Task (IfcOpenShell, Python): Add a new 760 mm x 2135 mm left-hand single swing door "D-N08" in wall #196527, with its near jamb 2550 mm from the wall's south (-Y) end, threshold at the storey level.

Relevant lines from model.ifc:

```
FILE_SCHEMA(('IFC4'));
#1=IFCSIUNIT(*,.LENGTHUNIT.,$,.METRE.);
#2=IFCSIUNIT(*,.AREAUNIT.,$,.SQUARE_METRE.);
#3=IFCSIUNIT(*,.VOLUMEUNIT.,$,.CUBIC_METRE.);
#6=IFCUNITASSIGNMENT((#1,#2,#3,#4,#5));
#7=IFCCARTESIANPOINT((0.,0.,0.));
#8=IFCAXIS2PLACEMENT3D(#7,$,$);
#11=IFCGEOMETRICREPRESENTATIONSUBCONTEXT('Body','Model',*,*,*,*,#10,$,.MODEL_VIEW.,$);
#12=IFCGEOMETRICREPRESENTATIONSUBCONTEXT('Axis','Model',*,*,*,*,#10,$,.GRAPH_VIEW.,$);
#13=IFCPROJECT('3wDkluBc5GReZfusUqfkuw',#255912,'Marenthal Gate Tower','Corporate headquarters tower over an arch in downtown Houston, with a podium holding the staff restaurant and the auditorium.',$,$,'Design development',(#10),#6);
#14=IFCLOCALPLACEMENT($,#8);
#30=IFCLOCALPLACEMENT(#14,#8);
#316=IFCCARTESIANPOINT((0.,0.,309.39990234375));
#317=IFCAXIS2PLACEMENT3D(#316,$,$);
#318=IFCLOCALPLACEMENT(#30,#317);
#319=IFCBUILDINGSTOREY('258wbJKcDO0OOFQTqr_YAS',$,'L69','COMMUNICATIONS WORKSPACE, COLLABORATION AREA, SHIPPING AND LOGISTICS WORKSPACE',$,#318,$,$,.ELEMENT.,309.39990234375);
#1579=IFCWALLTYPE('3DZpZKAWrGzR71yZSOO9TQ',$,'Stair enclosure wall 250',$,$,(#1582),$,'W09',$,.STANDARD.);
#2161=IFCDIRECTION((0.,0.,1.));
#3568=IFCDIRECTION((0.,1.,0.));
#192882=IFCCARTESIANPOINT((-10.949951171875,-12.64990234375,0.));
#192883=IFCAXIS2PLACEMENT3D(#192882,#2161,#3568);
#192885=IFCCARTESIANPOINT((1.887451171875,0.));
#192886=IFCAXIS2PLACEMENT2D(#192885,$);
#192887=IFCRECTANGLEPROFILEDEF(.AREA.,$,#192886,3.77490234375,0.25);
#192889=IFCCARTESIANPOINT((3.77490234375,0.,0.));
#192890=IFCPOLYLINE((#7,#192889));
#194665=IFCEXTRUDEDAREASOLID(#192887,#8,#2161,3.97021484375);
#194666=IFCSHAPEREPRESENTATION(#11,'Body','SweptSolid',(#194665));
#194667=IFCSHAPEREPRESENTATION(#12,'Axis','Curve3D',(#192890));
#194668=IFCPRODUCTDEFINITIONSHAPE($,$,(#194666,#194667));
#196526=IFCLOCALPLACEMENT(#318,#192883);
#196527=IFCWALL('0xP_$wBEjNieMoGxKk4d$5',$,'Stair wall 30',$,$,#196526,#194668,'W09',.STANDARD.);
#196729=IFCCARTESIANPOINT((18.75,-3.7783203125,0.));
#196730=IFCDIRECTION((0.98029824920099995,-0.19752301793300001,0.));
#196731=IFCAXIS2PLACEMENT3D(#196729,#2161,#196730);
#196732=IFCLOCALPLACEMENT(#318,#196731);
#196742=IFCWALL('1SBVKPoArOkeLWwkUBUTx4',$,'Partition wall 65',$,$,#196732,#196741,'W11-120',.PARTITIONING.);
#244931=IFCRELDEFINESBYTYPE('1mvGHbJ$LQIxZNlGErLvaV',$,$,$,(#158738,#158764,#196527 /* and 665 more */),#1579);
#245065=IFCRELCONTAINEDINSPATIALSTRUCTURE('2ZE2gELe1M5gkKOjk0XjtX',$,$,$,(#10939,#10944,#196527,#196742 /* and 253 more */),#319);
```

```python
import numpy as np
import ifcopenshell
import ifcopenshell.api.feature
import ifcopenshell.api.geometry
import ifcopenshell.api.root
import ifcopenshell.api.spatial
import ifcopenshell.geom
import ifcopenshell.util.element
import ifcopenshell.util.placement
import ifcopenshell.util.representation
import ifcopenshell.util.shape
import ifcopenshell.util.unit

model = ifcopenshell.open("model.ifc")
unit_scale = ifcopenshell.util.unit.calculate_unit_scale(model)
settings = ifcopenshell.geom.settings()


def volume(element):
    """Net volume in cubic metres, openings subtracted."""
    shape = ifcopenshell.geom.create_shape(settings, element)
    return ifcopenshell.util.shape.get_volume(shape.geometry)


wall = model.by_id(196527)
storey = ifcopenshell.util.element.get_container(wall, ifc_class="IfcBuildingStorey")
context = ifcopenshell.util.representation.get_context(model, "Model", "Body", "MODEL_VIEW")
before = volume(wall)

width, height, from_end, sill = 0.76, 2.135, 2.55, 0.0  # metres

# The wall runs along its own X axis, and the end named is its -X end.
wall_shape = ifcopenshell.geom.create_shape(settings, wall)
x, y, z = ifcopenshell.util.shape.get_vertices(wall_shape.geometry).T
start = x.min() + from_end
face, thickness = float(y.min()), float(y.max() - y.min())
wall_matrix = ifcopenshell.util.placement.get_local_placement(wall.ObjectPlacement)
level = ifcopenshell.util.placement.get_local_placement(storey.ObjectPlacement)[2, 3]


def in_wall(x, y):
    """Placement at x, y metres in the wall's axes, at sill height."""
    matrix = wall_matrix.copy()
    matrix[:, 3] = wall_matrix @ np.array([x / unit_scale, y / unit_scale, 0.0, 1.0])
    matrix[2, 3] = level + sill / unit_scale
    return matrix


# Opening: a box that overshoots both wall faces by 50 mm.
opening = ifcopenshell.api.root.create_entity(model, ifc_class="IfcOpeningElement", predefined_type="OPENING")
box = ifcopenshell.api.geometry.add_wall_representation(
    model, context=context, length=width, height=height, thickness=thickness + 0.1
)
ifcopenshell.api.geometry.assign_representation(model, product=opening, representation=box)
ifcopenshell.api.geometry.edit_object_placement(model, product=opening, matrix=in_wall(start, face - 0.05), is_si=False)
ifcopenshell.api.feature.add_feature(model, feature=opening, element=wall)

door = ifcopenshell.api.root.create_entity(model, ifc_class="IfcDoor", name="D-N08", predefined_type="DOOR")
door.OverallWidth, door.OverallHeight = width / unit_scale, height / unit_scale
door.OperationType = "SINGLE_SWING_LEFT"
body = ifcopenshell.api.geometry.add_door_representation(
    model,
    context=context,
    overall_width=door.OverallWidth,
    overall_height=door.OverallHeight,
    operation_type="SINGLE_SWING_LEFT",
    lining_properties={"LiningDepth": thickness / unit_scale, "ThresholdDepth": thickness / unit_scale},
)
ifcopenshell.api.geometry.assign_representation(model, product=door, representation=body)
ifcopenshell.api.spatial.assign_container(model, products=[door], relating_structure=storey)
ifcopenshell.api.feature.add_filling(model, opening=opening, element=door)

# The lining spans the wall, so the door starts at the wall face.
ifcopenshell.api.geometry.edit_object_placement(model, product=door, matrix=in_wall(start, face), is_si=False)

after = volume(wall)

print(f"wall volume {before:.3f} -> {after:.3f} m3")

model.write("model_rev.ifc")
```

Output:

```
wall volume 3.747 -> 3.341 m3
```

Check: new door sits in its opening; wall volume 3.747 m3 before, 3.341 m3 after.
